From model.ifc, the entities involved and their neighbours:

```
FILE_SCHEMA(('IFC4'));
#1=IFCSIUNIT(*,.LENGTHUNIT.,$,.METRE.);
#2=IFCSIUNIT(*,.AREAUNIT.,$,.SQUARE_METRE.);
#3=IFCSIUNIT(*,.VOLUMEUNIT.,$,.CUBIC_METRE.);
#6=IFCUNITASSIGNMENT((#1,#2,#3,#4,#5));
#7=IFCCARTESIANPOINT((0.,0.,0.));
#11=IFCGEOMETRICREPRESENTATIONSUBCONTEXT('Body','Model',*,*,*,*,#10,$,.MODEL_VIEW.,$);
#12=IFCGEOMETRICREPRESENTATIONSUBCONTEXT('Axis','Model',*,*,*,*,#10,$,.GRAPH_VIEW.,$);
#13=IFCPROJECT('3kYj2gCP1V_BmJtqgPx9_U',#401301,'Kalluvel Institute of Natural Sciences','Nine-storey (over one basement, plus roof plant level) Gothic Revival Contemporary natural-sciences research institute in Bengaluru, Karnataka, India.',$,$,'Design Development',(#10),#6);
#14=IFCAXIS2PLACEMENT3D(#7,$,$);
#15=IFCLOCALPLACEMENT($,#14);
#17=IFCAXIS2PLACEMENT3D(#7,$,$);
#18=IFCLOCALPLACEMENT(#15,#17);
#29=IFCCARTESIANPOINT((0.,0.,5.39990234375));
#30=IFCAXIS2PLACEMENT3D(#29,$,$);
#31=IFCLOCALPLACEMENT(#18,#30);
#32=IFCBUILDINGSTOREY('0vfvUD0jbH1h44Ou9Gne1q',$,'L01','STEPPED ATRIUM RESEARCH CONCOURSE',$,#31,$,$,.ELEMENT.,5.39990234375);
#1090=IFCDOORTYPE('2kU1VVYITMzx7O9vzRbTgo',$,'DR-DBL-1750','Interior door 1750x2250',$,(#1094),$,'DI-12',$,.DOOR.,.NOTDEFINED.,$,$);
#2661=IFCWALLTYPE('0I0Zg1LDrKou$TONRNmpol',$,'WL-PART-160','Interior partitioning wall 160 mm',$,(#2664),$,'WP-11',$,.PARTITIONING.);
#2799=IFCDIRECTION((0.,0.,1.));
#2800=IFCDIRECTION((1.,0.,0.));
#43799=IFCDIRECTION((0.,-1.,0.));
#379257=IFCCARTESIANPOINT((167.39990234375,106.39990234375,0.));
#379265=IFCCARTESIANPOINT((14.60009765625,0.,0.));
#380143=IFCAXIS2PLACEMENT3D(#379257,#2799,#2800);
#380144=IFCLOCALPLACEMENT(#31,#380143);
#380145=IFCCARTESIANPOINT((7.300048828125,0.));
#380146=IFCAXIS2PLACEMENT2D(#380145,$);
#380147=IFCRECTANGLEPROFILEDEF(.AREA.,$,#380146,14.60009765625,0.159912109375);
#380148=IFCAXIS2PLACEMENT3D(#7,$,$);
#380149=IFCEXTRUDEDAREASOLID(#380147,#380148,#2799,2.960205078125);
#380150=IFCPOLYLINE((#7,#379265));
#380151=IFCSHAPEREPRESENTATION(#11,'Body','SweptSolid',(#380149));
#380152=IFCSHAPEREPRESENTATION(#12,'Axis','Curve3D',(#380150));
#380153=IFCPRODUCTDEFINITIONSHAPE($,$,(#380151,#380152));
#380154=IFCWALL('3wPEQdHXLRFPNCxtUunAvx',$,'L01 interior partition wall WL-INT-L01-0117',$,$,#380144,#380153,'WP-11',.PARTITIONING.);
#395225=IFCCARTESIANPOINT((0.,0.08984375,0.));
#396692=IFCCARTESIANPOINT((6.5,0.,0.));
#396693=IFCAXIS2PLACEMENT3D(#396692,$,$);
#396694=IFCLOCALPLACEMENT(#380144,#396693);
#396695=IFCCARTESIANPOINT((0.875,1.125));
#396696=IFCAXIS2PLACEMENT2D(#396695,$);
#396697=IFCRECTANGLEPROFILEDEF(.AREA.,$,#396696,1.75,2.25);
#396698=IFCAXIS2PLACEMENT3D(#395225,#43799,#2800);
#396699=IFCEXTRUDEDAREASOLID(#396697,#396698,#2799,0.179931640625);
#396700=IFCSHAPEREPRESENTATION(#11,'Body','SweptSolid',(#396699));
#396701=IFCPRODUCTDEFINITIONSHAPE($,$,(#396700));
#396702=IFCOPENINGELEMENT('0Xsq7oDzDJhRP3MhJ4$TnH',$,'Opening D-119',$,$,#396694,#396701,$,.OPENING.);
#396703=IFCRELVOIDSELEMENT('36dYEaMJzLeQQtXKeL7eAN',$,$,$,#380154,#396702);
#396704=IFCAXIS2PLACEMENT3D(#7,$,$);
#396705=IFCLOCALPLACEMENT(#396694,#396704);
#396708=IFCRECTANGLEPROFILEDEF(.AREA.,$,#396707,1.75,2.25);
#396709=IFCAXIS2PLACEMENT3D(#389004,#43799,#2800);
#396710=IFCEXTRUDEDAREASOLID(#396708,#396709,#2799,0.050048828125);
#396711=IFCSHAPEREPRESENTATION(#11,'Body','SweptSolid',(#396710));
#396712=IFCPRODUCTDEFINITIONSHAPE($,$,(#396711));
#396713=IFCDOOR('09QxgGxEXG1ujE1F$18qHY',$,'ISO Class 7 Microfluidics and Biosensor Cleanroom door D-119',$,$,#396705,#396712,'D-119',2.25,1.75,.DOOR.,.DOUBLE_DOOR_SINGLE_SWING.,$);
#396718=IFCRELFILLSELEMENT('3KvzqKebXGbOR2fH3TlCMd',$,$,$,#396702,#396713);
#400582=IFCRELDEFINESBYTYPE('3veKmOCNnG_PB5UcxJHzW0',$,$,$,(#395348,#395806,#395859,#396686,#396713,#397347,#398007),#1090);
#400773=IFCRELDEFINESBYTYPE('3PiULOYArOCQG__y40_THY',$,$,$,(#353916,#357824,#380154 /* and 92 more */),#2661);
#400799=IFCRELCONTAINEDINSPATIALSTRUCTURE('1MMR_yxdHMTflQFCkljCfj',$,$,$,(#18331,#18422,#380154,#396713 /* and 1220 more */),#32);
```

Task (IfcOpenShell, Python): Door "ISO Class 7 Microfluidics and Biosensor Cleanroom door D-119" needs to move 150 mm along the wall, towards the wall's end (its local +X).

```python
import ifcopenshell
import ifcopenshell.api.geometry
import ifcopenshell.util.placement

model = ifcopenshell.open("model.ifc")

door = model.by_id(396713)
opening = door.FillsVoids[0].RelatingOpeningElement
wall = opening.VoidsElements[0].RelatingBuildingElement

wall_matrix = ifcopenshell.util.placement.get_local_placement(wall.ObjectPlacement)
shift = wall_matrix[:3, 0] * 0.15
before = ifcopenshell.util.placement.get_local_placement(door.ObjectPlacement)[:3, 3].copy()

# The door is placed relative to its opening, so it follows when the opening moves.
matrix = ifcopenshell.util.placement.get_local_placement(opening.ObjectPlacement)
matrix[:3, 3] += shift
ifcopenshell.api.geometry.edit_object_placement(
    model, product=opening, matrix=matrix, is_si=False, should_transform_children=True
)

after = ifcopenshell.util.placement.get_local_placement(door.ObjectPlacement)[:3, 3]
print("door moved by", (after - before).round(3) + 0.0)

model.write("model-out.ifc")
```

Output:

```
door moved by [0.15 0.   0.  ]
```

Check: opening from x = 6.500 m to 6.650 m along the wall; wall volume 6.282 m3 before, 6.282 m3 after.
